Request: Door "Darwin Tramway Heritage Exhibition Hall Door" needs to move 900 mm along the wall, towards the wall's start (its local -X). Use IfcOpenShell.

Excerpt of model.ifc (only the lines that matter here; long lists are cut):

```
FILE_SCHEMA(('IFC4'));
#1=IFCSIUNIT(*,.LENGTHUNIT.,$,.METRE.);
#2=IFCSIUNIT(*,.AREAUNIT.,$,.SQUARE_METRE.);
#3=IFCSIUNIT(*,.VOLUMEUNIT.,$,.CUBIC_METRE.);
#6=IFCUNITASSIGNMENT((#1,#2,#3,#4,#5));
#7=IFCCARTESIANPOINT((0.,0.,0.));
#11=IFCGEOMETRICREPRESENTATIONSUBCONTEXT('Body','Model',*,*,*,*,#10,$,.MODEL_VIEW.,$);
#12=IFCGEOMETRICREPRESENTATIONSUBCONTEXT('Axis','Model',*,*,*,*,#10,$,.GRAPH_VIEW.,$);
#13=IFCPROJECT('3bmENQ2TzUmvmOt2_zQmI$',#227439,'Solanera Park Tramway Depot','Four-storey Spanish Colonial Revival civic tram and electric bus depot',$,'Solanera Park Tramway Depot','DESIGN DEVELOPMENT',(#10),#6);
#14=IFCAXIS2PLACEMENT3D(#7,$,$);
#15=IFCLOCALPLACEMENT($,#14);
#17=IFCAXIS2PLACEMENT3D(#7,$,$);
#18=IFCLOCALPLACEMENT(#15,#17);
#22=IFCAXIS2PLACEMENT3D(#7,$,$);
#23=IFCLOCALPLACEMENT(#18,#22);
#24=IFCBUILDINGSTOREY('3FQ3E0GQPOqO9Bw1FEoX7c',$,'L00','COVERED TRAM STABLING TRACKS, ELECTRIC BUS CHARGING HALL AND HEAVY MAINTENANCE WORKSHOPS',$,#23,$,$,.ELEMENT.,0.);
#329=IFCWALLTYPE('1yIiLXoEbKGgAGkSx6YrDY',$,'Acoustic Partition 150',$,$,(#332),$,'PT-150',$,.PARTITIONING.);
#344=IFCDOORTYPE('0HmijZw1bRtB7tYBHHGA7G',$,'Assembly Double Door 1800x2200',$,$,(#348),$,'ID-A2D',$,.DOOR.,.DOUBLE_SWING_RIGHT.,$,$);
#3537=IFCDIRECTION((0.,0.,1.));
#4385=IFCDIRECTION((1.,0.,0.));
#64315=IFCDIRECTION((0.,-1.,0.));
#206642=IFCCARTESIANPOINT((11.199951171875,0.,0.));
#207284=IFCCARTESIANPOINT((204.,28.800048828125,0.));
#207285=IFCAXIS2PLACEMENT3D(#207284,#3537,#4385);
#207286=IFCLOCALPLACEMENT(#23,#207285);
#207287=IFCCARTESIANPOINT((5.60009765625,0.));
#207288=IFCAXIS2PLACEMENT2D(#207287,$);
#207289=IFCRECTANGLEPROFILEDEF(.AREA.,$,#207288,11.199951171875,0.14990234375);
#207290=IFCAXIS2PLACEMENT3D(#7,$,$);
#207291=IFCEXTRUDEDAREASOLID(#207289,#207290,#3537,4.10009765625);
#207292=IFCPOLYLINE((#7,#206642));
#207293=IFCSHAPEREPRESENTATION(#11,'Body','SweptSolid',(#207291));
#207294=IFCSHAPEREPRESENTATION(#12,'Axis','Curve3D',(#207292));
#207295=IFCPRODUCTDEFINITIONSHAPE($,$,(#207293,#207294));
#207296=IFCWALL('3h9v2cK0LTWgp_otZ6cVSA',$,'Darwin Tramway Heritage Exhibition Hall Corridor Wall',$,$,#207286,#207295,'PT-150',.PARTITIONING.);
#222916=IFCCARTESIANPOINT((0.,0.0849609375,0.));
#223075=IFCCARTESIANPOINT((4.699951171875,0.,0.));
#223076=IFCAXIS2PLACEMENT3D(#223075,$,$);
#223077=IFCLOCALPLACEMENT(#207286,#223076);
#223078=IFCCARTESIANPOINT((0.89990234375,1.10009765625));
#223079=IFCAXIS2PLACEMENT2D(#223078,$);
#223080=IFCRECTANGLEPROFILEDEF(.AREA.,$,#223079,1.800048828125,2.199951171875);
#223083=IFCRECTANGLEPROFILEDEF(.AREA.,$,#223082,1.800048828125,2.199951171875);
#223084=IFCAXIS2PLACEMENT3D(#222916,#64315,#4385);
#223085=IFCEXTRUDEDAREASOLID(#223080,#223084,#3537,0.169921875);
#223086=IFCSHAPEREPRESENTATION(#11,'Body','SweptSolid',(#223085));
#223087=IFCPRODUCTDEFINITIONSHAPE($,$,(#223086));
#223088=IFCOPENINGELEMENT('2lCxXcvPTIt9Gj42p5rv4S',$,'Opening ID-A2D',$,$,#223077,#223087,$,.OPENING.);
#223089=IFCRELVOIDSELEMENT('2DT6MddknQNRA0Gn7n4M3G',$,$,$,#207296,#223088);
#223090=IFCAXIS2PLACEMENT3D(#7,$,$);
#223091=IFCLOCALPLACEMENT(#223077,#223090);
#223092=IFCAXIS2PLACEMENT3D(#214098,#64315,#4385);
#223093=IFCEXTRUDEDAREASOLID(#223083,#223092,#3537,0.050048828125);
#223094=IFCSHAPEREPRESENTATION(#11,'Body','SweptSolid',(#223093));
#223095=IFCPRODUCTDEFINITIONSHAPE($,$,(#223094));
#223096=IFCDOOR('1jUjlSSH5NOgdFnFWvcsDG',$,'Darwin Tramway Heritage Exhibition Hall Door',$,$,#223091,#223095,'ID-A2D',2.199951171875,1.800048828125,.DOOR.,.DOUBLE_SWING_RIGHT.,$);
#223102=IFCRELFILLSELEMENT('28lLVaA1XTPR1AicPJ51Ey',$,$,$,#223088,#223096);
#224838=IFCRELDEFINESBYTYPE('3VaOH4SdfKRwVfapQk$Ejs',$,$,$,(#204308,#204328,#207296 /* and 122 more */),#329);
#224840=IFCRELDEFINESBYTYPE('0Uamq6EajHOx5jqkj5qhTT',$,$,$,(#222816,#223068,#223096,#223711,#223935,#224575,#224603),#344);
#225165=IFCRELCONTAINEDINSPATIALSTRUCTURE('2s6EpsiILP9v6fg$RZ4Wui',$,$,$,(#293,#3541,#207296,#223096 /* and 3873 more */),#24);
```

```python
import ifcopenshell
import ifcopenshell.api.geometry
import ifcopenshell.util.placement
import ifcopenshell.util.unit

model = ifcopenshell.open("model.ifc")
unit_scale = ifcopenshell.util.unit.calculate_unit_scale(model)

door = model.by_id(223096)
opening = door.FillsVoids[0].RelatingOpeningElement
wall = opening.VoidsElements[0].RelatingBuildingElement

wall_matrix = ifcopenshell.util.placement.get_local_placement(wall.ObjectPlacement)
shift = wall_matrix[:3, 0] * -0.9 / unit_scale
before = ifcopenshell.util.placement.get_local_placement(door.ObjectPlacement)[:3, 3].copy()

# The door is placed relative to its opening, so it follows when the opening moves.
matrix = ifcopenshell.util.placement.get_local_placement(opening.ObjectPlacement)
matrix[:3, 3] += shift
ifcopenshell.api.geometry.edit_object_placement(
    model, product=opening, matrix=matrix, is_si=False, should_transform_children=True
)

after = ifcopenshell.util.placement.get_local_placement(door.ObjectPlacement)[:3, 3]
print("door moved by", (after - before).round(3) + 0.0)

model.write("model_edited.ifc")
```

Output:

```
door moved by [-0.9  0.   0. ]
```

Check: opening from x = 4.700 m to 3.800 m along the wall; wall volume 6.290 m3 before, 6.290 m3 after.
